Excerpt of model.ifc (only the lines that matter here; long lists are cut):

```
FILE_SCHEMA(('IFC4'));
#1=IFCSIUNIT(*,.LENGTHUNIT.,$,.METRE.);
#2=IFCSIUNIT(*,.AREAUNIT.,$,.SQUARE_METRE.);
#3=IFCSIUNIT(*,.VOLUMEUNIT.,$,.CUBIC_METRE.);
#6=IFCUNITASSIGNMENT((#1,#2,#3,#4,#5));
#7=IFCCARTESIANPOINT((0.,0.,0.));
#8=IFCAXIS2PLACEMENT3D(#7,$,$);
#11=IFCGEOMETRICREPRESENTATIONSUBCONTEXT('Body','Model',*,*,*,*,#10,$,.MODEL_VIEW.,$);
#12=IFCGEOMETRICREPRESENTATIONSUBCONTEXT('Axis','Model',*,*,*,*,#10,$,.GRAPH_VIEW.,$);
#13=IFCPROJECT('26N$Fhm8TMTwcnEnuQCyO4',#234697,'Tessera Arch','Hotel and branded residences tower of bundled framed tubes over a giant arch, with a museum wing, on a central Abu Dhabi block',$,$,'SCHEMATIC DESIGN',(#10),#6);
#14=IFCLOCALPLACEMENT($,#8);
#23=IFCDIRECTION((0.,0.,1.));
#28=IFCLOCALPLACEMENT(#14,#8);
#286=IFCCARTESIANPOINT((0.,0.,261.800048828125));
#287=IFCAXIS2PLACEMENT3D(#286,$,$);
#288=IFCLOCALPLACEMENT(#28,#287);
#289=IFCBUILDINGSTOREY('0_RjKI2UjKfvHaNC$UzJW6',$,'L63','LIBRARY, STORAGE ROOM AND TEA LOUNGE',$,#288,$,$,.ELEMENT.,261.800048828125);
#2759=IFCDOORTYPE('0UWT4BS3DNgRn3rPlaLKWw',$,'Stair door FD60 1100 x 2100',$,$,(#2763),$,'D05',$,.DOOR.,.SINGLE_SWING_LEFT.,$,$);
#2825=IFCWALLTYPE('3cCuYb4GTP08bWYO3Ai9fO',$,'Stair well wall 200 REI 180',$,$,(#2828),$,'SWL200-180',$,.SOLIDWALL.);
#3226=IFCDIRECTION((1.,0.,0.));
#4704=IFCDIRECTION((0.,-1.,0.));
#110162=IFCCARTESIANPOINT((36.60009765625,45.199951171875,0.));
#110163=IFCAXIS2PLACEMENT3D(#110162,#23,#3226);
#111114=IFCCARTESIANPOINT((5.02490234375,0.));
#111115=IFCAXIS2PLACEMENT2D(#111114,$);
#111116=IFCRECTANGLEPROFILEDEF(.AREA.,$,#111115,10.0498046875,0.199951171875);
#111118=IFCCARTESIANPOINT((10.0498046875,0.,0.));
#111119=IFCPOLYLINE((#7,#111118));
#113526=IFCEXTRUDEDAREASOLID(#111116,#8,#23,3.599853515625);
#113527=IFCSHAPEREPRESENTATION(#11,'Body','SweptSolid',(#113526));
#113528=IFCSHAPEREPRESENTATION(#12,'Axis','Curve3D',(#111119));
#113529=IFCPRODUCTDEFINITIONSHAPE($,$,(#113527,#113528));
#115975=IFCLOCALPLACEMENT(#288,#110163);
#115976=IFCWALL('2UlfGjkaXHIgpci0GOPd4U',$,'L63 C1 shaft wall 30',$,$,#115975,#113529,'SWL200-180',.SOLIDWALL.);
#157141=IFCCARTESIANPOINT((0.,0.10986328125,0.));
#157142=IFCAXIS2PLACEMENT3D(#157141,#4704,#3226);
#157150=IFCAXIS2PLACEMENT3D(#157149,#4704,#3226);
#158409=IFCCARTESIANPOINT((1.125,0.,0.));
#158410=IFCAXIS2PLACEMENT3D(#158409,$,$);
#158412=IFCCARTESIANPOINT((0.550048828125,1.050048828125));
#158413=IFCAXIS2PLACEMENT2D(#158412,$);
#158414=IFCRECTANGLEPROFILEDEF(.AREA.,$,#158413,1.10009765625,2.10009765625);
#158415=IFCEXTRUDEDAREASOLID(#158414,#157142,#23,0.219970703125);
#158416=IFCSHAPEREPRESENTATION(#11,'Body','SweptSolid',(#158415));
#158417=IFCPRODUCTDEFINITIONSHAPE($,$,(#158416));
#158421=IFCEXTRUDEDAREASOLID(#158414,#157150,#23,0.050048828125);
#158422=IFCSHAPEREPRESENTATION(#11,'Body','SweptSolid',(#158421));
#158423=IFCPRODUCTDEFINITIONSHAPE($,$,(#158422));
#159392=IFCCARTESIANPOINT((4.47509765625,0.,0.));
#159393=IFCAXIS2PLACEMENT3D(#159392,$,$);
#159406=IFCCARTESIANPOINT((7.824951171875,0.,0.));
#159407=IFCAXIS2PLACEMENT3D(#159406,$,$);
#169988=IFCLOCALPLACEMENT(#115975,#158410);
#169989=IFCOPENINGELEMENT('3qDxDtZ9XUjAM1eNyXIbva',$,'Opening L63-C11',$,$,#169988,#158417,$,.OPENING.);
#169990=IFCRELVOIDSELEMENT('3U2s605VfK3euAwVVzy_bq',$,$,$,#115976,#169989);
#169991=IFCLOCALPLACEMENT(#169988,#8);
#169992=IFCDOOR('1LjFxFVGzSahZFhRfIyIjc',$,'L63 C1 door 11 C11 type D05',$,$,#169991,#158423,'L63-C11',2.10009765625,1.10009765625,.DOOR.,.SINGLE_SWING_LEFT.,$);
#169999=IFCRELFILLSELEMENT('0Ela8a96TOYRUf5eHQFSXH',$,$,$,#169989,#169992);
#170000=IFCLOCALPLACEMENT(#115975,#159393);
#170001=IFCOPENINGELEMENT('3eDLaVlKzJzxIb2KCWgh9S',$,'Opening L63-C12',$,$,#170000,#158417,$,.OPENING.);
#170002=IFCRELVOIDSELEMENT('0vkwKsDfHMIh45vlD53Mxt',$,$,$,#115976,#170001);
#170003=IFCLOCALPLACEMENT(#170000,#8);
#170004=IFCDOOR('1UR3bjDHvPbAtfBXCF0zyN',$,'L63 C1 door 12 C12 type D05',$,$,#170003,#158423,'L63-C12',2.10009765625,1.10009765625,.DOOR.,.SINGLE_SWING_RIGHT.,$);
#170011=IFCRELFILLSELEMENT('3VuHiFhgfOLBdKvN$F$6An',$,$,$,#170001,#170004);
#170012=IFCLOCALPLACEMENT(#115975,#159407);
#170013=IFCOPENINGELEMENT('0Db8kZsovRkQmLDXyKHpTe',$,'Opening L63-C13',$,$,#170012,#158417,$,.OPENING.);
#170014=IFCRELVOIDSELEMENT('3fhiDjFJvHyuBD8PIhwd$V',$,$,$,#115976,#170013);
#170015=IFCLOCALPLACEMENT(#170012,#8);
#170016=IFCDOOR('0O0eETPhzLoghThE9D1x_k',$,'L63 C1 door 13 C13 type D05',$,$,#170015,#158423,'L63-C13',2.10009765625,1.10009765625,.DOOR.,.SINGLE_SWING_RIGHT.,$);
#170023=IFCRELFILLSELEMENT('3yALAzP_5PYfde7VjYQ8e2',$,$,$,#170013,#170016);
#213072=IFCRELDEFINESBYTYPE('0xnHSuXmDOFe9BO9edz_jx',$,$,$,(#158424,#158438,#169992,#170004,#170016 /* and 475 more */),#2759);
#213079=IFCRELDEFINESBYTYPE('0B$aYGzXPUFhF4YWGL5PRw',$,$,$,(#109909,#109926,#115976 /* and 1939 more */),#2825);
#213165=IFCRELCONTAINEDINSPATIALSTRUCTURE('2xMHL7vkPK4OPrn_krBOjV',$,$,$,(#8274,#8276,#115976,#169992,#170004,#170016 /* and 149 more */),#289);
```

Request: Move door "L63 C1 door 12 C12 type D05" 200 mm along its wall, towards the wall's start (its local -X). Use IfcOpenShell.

```python
import ifcopenshell
import ifcopenshell.api.geometry
import ifcopenshell.util.placement
import ifcopenshell.util.unit

model = ifcopenshell.open("model.ifc")
unit_scale = ifcopenshell.util.unit.calculate_unit_scale(model)

door = model.by_guid("1UR3bjDHvPbAtfBXCF0zyN")
opening = door.FillsVoids[0].RelatingOpeningElement
wall = opening.VoidsElements[0].RelatingBuildingElement

wall_matrix = ifcopenshell.util.placement.get_local_placement(wall.ObjectPlacement)
shift = wall_matrix[:3, 0] * -0.2 / unit_scale
before = ifcopenshell.util.placement.get_local_placement(door.ObjectPlacement)[:3, 3].copy()

# The door is placed relative to its opening, so it follows when the opening moves.
matrix = ifcopenshell.util.placement.get_local_placement(opening.ObjectPlacement)
matrix[:3, 3] += shift
ifcopenshell.api.geometry.edit_object_placement(
    model, product=opening, matrix=matrix, is_si=False, should_transform_children=True
)

after = ifcopenshell.util.placement.get_local_placement(door.ObjectPlacement)[:3, 3]
print("door moved by", (after - before).round(3) + 0.0)

model.write("model_edited.ifc")
```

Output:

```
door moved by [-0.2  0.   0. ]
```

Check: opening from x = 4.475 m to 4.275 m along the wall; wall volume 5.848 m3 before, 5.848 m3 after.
